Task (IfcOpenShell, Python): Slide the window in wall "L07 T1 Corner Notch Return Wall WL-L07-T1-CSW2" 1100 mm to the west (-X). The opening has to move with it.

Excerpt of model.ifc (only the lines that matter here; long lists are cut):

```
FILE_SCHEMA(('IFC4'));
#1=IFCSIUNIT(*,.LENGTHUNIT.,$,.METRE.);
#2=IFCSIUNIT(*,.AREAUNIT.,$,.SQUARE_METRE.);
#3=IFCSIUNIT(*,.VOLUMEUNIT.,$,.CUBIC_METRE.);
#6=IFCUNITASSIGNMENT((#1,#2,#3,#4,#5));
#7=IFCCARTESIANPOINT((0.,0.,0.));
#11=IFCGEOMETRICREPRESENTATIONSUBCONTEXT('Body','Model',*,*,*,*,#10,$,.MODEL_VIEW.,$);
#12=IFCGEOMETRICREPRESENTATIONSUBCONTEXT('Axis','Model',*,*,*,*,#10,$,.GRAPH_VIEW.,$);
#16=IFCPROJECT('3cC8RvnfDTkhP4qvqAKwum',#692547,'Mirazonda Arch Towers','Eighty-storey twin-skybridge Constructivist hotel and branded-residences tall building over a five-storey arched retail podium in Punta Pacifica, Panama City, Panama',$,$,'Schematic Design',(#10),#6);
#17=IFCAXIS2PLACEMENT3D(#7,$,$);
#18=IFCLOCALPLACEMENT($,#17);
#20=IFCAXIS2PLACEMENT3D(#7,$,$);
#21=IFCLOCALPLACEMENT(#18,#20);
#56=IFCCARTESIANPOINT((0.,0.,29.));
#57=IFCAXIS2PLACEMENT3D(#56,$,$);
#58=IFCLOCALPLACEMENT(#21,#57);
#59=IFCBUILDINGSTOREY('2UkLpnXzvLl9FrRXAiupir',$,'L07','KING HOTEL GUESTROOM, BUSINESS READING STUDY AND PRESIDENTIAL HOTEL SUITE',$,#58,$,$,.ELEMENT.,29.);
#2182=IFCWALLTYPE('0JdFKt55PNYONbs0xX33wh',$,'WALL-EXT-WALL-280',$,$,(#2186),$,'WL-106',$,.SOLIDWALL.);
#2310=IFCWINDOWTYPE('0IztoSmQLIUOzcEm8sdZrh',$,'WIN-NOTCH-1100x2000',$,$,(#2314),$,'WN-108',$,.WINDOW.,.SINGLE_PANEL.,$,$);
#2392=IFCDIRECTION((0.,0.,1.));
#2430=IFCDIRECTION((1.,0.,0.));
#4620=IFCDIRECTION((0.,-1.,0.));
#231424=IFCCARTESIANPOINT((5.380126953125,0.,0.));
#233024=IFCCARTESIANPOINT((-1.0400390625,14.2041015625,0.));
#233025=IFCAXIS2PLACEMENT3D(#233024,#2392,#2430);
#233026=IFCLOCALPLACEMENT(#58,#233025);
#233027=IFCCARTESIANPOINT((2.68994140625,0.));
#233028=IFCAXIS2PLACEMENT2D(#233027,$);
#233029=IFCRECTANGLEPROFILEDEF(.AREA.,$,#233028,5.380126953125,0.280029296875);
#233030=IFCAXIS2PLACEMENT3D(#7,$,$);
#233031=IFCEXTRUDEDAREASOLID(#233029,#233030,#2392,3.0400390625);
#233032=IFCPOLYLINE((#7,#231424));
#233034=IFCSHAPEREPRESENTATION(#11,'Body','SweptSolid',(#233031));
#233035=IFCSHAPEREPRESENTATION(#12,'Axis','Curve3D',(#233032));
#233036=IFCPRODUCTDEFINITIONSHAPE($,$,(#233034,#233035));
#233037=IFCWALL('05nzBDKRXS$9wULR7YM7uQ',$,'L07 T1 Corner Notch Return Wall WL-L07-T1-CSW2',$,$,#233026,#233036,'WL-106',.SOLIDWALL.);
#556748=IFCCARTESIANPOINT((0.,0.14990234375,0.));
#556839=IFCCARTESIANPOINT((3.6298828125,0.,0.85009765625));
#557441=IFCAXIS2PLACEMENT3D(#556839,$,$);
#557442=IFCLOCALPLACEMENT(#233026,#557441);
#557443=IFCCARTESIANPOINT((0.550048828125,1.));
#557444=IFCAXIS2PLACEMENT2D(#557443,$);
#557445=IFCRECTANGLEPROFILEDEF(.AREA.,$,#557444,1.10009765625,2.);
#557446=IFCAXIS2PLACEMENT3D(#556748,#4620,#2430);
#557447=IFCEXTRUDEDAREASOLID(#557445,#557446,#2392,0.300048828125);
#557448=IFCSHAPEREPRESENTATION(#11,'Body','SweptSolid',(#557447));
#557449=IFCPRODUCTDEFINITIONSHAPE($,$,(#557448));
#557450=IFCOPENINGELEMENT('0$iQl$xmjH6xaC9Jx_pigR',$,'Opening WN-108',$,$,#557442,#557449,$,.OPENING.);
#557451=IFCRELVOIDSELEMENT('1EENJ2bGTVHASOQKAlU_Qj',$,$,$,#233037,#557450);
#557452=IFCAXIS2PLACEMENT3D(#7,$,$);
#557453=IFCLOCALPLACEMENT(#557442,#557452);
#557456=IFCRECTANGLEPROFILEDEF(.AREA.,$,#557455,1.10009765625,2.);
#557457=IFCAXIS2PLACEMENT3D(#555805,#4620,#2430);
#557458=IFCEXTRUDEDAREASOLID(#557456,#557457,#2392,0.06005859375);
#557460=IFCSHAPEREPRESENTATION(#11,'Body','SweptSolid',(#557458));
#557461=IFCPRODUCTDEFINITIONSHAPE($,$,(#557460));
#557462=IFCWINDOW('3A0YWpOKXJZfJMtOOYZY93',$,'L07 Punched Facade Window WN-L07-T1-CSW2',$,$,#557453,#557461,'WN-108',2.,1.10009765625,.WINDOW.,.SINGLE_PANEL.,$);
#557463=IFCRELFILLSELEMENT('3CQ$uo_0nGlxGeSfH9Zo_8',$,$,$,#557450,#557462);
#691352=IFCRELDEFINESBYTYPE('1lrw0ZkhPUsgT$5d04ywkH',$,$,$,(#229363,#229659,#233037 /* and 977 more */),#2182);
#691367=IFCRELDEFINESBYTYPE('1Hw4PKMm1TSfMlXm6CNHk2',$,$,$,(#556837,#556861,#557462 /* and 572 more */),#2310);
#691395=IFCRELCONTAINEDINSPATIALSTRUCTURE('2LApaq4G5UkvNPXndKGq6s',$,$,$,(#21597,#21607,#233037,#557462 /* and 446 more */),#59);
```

```python
import ifcopenshell
import ifcopenshell.api.geometry
import ifcopenshell.util.placement
import ifcopenshell.util.unit

model = ifcopenshell.open("model.ifc")
unit_scale = ifcopenshell.util.unit.calculate_unit_scale(model)

window = model.by_guid("3A0YWpOKXJZfJMtOOYZY93")
opening = window.FillsVoids[0].RelatingOpeningElement
wall = opening.VoidsElements[0].RelatingBuildingElement

wall_matrix = ifcopenshell.util.placement.get_local_placement(wall.ObjectPlacement)
shift = wall_matrix[:3, 0] * -1.1 / unit_scale
before = ifcopenshell.util.placement.get_local_placement(window.ObjectPlacement)[:3, 3].copy()

# The window is placed relative to its opening, so it follows when the opening moves.
matrix = ifcopenshell.util.placement.get_local_placement(opening.ObjectPlacement)
matrix[:3, 3] += shift
ifcopenshell.api.geometry.edit_object_placement(
    model, product=opening, matrix=matrix, is_si=False, should_transform_children=True
)

after = ifcopenshell.util.placement.get_local_placement(window.ObjectPlacement)[:3, 3]
print("window moved by", (after - before).round(3) + 0.0)

model.write("model-out.ifc")
```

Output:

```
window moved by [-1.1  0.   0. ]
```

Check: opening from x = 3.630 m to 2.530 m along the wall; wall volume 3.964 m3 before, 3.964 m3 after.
